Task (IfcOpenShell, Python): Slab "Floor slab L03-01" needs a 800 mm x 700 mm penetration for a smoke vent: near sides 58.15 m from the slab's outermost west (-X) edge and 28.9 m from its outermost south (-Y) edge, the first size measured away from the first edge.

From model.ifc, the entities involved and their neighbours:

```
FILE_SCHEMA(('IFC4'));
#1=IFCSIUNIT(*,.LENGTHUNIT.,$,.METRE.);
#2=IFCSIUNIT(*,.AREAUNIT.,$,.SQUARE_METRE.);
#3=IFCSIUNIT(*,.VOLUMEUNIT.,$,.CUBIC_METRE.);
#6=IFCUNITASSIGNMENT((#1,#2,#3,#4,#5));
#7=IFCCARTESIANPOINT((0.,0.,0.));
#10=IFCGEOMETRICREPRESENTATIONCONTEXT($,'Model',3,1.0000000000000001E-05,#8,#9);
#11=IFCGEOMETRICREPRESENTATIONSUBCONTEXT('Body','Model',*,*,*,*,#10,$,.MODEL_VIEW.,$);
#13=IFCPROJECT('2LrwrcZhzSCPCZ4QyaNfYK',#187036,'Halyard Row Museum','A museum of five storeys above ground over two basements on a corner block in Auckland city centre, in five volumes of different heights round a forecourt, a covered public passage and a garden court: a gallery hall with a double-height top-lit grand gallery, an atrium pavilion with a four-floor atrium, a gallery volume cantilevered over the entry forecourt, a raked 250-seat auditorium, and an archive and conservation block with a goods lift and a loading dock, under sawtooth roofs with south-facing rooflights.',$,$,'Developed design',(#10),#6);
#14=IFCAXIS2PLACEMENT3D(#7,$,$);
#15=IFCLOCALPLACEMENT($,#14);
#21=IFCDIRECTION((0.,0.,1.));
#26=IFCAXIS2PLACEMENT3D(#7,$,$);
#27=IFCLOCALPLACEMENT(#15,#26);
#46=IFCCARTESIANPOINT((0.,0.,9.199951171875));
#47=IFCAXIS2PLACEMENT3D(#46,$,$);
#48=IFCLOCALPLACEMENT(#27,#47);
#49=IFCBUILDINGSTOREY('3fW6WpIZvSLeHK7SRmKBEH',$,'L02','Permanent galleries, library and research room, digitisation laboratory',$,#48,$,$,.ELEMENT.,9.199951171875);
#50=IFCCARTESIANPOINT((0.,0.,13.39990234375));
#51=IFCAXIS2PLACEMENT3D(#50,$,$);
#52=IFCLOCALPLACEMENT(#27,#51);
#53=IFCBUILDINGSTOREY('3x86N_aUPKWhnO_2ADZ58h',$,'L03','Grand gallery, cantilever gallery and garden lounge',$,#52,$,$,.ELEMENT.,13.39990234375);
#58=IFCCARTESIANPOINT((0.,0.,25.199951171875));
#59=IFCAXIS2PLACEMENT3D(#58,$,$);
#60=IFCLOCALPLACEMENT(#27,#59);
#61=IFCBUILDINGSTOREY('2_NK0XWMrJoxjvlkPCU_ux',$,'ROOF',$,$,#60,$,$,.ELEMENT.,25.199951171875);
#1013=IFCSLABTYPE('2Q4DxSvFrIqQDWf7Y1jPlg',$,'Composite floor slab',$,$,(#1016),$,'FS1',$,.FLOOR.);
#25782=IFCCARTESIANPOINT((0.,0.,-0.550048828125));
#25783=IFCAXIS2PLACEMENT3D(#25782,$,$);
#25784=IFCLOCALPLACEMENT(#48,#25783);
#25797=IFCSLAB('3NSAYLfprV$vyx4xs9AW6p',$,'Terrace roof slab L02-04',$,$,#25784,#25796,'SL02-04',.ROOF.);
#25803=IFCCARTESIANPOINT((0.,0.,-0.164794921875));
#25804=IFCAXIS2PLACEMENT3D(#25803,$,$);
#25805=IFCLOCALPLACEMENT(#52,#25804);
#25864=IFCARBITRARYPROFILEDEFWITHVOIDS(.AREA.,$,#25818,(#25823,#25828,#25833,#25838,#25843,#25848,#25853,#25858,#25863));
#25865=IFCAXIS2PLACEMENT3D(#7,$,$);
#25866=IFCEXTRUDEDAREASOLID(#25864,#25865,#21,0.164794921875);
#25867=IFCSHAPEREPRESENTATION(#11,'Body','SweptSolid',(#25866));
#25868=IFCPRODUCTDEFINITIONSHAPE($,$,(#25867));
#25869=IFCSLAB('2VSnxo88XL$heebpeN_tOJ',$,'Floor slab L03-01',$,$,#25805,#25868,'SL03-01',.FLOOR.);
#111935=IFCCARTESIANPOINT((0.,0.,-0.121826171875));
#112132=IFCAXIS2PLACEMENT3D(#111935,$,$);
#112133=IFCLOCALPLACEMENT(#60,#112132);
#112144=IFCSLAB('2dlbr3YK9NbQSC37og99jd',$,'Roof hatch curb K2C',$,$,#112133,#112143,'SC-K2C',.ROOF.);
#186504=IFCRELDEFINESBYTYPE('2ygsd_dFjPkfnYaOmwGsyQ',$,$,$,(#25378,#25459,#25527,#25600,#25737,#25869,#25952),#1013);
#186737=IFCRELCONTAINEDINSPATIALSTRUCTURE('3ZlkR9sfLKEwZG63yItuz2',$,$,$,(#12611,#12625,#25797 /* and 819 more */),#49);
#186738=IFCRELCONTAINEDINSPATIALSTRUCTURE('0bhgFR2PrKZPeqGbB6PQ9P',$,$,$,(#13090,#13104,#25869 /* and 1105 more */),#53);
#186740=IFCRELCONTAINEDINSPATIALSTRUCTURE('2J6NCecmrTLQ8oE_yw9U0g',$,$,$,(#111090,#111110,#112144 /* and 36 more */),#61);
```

```python
import numpy as np
import ifcopenshell
import ifcopenshell.api.feature
import ifcopenshell.api.geometry
import ifcopenshell.api.root
import ifcopenshell.geom
import ifcopenshell.util.placement
import ifcopenshell.util.representation
import ifcopenshell.util.shape
import ifcopenshell.util.unit

model = ifcopenshell.open("model.ifc")
unit_scale = ifcopenshell.util.unit.calculate_unit_scale(model)
settings = ifcopenshell.geom.settings()


def volume(element):
    """Net volume in cubic metres, openings subtracted."""
    shape = ifcopenshell.geom.create_shape(settings, element)
    return ifcopenshell.util.shape.get_volume(shape.geometry)


slab = model.by_guid("2VSnxo88XL$heebpeN_tOJ")
before = volume(slab)

# Extent in the slab's own axes, in metres. The edges named are its -X and -Y sides.
slab_shape = ifcopenshell.geom.create_shape(settings, slab)
vertices = ifcopenshell.util.shape.get_vertices(slab_shape.geometry)
x_min, y_min, bottom = vertices.min(axis=0)
top = vertices[:, 2].max()

opening = ifcopenshell.api.root.create_entity(model, ifc_class="IfcOpeningElement", name="Smoke vent opening", predefined_type="OPENING")
context = ifcopenshell.util.representation.get_context(model, "Model", "Body", "MODEL_VIEW")
width, depth = 0.8, 0.7
outline = [(0.0, 0.0), (width, 0.0), (width, depth), (0.0, depth), (0.0, 0.0)]
# Overshoot both faces by 50 mm so the cut is clean.
shape = ifcopenshell.api.geometry.add_slab_representation(
    model, context=context, depth=top - bottom + 0.1, polyline=outline
)
ifcopenshell.api.geometry.assign_representation(model, product=opening, representation=shape)

matrix = ifcopenshell.util.placement.get_local_placement(slab.ObjectPlacement)
matrix[:, 3] = matrix @ np.append(np.array([x_min + 58.15, y_min + 28.9, bottom - 0.05]) / unit_scale, 1.0)
ifcopenshell.api.geometry.edit_object_placement(model, product=opening, matrix=matrix, is_si=False)
ifcopenshell.api.feature.add_feature(model, feature=opening, element=slab)

after = volume(slab)

print(f"slab volume {before:.3f} -> {after:.3f} m3")

model.write("model_updated.ifc")
```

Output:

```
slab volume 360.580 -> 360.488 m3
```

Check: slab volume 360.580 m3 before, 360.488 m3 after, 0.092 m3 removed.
